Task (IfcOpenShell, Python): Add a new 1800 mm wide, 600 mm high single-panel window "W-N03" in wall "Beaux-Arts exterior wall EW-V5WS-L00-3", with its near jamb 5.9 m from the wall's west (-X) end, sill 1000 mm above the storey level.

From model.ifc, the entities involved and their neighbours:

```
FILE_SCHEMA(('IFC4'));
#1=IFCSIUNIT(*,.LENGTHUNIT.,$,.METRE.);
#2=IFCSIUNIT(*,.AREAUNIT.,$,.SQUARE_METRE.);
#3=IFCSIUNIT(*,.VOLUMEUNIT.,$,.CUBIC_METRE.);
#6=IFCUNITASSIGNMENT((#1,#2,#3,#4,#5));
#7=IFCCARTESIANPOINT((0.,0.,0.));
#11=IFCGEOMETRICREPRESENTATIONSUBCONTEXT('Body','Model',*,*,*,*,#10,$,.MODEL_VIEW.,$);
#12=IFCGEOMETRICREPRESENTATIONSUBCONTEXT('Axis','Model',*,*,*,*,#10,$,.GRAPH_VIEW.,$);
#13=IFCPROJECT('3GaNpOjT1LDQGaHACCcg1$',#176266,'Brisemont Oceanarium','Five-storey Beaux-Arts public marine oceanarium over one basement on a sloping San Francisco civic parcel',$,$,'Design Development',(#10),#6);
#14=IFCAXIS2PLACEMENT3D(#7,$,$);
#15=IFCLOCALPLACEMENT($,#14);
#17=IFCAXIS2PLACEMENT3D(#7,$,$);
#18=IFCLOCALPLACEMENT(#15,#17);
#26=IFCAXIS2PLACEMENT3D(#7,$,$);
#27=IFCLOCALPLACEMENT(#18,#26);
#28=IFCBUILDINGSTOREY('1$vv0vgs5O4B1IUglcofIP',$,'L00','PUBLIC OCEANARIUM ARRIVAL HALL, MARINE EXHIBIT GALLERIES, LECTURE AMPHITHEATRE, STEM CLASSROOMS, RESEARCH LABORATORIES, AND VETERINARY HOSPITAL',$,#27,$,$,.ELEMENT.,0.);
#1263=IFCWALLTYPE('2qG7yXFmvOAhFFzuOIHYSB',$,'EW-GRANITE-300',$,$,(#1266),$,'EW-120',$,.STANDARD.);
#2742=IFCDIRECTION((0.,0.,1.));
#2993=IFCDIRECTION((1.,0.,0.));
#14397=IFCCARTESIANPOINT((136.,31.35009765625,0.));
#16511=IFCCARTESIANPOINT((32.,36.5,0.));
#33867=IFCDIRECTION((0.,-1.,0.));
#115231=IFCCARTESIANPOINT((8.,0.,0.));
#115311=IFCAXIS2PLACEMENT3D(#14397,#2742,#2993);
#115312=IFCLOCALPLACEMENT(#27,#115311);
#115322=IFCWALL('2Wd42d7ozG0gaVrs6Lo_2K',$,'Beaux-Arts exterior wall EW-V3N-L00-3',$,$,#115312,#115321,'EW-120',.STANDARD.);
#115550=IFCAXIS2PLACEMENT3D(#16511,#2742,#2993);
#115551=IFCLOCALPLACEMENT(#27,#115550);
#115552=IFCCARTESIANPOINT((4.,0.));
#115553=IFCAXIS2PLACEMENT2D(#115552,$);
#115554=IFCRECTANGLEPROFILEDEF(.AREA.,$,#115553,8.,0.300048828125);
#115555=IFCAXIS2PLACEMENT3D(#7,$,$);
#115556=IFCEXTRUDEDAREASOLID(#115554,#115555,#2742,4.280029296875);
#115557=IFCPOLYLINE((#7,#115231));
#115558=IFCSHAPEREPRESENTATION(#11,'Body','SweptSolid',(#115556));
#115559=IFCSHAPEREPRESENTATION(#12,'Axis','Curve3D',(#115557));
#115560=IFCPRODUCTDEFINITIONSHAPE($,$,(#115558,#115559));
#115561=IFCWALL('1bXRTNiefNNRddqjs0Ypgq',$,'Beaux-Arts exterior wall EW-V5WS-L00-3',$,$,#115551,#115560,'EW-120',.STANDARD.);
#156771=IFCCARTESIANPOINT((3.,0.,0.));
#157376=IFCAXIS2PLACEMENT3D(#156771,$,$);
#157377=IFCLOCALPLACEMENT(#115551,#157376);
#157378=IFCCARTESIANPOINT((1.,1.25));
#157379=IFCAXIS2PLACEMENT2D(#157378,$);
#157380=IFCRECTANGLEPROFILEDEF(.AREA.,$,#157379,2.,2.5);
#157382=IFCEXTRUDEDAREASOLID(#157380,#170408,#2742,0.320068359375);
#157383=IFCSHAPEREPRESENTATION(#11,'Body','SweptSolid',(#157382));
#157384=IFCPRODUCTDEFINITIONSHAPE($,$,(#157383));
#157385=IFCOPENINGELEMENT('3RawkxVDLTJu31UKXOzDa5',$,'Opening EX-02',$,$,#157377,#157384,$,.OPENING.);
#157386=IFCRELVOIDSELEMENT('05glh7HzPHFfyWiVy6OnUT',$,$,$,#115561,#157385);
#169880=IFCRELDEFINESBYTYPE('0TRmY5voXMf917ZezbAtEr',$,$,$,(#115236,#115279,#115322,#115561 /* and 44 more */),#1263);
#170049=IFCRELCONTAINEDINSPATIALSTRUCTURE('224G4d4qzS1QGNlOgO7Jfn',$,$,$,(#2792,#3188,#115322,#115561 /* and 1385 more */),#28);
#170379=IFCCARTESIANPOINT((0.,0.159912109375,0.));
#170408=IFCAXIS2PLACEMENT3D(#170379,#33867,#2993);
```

```python
import numpy as np
import ifcopenshell
import ifcopenshell.api.feature
import ifcopenshell.api.geometry
import ifcopenshell.api.root
import ifcopenshell.api.spatial
import ifcopenshell.geom
import ifcopenshell.util.element
import ifcopenshell.util.placement
import ifcopenshell.util.representation
import ifcopenshell.util.shape
import ifcopenshell.util.unit

model = ifcopenshell.open("model.ifc")
unit_scale = ifcopenshell.util.unit.calculate_unit_scale(model)
settings = ifcopenshell.geom.settings()


def volume(element):
    """Net volume in cubic metres, openings subtracted."""
    shape = ifcopenshell.geom.create_shape(settings, element)
    return ifcopenshell.util.shape.get_volume(shape.geometry)


wall = model.by_guid("1bXRTNiefNNRddqjs0Ypgq")
storey = ifcopenshell.util.element.get_container(wall, ifc_class="IfcBuildingStorey")
context = ifcopenshell.util.representation.get_context(model, "Model", "Body", "MODEL_VIEW")
before = volume(wall)

width, height, from_end, sill = 1.8, 0.6, 5.9, 1  # metres

# The wall runs along its own X axis, and the end named is its -X end.
wall_shape = ifcopenshell.geom.create_shape(settings, wall)
x, y, z = ifcopenshell.util.shape.get_vertices(wall_shape.geometry).T
start = x.min() + from_end
face, thickness = float(y.min()), float(y.max() - y.min())
wall_matrix = ifcopenshell.util.placement.get_local_placement(wall.ObjectPlacement)
level = ifcopenshell.util.placement.get_local_placement(storey.ObjectPlacement)[2, 3]


def in_wall(x, y):
    """Placement at x, y metres in the wall's axes, at sill height."""
    matrix = wall_matrix.copy()
    matrix[:, 3] = wall_matrix @ np.array([x / unit_scale, y / unit_scale, 0.0, 1.0])
    matrix[2, 3] = level + sill / unit_scale
    return matrix


# Opening: a box that overshoots both wall faces by 50 mm.
opening = ifcopenshell.api.root.create_entity(model, ifc_class="IfcOpeningElement", predefined_type="OPENING")
box = ifcopenshell.api.geometry.add_wall_representation(
    model, context=context, length=width, height=height, thickness=thickness + 0.1
)
ifcopenshell.api.geometry.assign_representation(model, product=opening, representation=box)
ifcopenshell.api.geometry.edit_object_placement(model, product=opening, matrix=in_wall(start, face - 0.05), is_si=False)
ifcopenshell.api.feature.add_feature(model, feature=opening, element=wall)

window = ifcopenshell.api.root.create_entity(model, ifc_class="IfcWindow", name="W-N03", predefined_type="WINDOW")
window.OverallWidth, window.OverallHeight = width / unit_scale, height / unit_scale
window.PartitioningType = "SINGLE_PANEL"
body = ifcopenshell.api.geometry.add_window_representation(
    model,
    context=context,
    overall_width=window.OverallWidth,
    overall_height=window.OverallHeight,
    partition_type="SINGLE_PANEL",
)
ifcopenshell.api.geometry.assign_representation(model, product=window, representation=body)
ifcopenshell.api.spatial.assign_container(model, products=[window], relating_structure=storey)
ifcopenshell.api.feature.add_filling(model, opening=opening, element=window)

# Centre the window in the wall's thickness.
ifcopenshell.api.geometry.edit_object_placement(model, product=window, matrix=in_wall(start, face), is_si=False)
window_shape = ifcopenshell.geom.create_shape(settings, window)
depth = ifcopenshell.util.shape.get_vertices(window_shape.geometry)[:, 1]
offset = face + thickness / 2 - (depth.min() + depth.max()) / 2
ifcopenshell.api.geometry.edit_object_placement(model, product=window, matrix=in_wall(start, offset), is_si=False)

after = volume(wall)

print(f"wall volume {before:.3f} -> {after:.3f} m3")

model.write("model_updated.ifc")
```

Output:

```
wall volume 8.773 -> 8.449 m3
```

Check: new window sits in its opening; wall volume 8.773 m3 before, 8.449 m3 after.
